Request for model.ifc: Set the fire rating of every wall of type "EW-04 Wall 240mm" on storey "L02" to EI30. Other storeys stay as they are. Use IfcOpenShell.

First a look at what the model holds.

```python
import ifcopenshell
import ifcopenshell.util.element

model = ifcopenshell.open("model.ifc")
print(model.schema)
storey = next(s for s in model.by_type("IfcBuildingStorey") if s.Name == "L02")
walls = [e for e in ifcopenshell.util.element.get_decomposition(storey) if e.is_a("IfcWall")]
seen = {}
for e in walls:
    element_type = ifcopenshell.util.element.get_type(e)
    key = (element_type.Name if element_type != e and element_type else None, ifcopenshell.util.element.get_pset(e, "Pset_WallCommon", "FireRating"))
    seen[key] = seen.get(key, 0) + 1
for (name, value), count in sorted(seen.items(), key=str):
    print(count, "x", name, "|", value)
```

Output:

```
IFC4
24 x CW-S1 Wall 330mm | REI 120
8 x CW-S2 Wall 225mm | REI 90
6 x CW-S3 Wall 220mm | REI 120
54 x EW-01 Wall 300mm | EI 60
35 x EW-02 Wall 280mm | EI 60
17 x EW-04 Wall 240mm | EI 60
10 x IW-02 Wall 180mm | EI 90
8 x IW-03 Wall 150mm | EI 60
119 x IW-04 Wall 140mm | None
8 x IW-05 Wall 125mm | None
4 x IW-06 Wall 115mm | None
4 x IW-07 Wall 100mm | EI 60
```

```python
import ifcopenshell
import ifcopenshell.api.pset
import ifcopenshell.util.element

model = ifcopenshell.open("model.ifc")

storey = next(s for s in model.by_type("IfcBuildingStorey") if s.Name == "L02")
walls = [e for e in ifcopenshell.util.element.get_decomposition(storey) if e.is_a("IfcWall")]

count = 0
for e in walls:
    element_type = ifcopenshell.util.element.get_type(e)
    if element_type in (None, e) or element_type.Name != "EW-04 Wall 240mm":
        continue
    # add_pset returns the element's existing set when there is one.
    pset = ifcopenshell.api.pset.add_pset(model, product=e, name="Pset_WallCommon")
    ifcopenshell.api.pset.edit_pset(model, pset=pset, properties={"FireRating": "EI30"})
    count += 1

print(count, "walls updated")

model.write("model_edited.ifc")
```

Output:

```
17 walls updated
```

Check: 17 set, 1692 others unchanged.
